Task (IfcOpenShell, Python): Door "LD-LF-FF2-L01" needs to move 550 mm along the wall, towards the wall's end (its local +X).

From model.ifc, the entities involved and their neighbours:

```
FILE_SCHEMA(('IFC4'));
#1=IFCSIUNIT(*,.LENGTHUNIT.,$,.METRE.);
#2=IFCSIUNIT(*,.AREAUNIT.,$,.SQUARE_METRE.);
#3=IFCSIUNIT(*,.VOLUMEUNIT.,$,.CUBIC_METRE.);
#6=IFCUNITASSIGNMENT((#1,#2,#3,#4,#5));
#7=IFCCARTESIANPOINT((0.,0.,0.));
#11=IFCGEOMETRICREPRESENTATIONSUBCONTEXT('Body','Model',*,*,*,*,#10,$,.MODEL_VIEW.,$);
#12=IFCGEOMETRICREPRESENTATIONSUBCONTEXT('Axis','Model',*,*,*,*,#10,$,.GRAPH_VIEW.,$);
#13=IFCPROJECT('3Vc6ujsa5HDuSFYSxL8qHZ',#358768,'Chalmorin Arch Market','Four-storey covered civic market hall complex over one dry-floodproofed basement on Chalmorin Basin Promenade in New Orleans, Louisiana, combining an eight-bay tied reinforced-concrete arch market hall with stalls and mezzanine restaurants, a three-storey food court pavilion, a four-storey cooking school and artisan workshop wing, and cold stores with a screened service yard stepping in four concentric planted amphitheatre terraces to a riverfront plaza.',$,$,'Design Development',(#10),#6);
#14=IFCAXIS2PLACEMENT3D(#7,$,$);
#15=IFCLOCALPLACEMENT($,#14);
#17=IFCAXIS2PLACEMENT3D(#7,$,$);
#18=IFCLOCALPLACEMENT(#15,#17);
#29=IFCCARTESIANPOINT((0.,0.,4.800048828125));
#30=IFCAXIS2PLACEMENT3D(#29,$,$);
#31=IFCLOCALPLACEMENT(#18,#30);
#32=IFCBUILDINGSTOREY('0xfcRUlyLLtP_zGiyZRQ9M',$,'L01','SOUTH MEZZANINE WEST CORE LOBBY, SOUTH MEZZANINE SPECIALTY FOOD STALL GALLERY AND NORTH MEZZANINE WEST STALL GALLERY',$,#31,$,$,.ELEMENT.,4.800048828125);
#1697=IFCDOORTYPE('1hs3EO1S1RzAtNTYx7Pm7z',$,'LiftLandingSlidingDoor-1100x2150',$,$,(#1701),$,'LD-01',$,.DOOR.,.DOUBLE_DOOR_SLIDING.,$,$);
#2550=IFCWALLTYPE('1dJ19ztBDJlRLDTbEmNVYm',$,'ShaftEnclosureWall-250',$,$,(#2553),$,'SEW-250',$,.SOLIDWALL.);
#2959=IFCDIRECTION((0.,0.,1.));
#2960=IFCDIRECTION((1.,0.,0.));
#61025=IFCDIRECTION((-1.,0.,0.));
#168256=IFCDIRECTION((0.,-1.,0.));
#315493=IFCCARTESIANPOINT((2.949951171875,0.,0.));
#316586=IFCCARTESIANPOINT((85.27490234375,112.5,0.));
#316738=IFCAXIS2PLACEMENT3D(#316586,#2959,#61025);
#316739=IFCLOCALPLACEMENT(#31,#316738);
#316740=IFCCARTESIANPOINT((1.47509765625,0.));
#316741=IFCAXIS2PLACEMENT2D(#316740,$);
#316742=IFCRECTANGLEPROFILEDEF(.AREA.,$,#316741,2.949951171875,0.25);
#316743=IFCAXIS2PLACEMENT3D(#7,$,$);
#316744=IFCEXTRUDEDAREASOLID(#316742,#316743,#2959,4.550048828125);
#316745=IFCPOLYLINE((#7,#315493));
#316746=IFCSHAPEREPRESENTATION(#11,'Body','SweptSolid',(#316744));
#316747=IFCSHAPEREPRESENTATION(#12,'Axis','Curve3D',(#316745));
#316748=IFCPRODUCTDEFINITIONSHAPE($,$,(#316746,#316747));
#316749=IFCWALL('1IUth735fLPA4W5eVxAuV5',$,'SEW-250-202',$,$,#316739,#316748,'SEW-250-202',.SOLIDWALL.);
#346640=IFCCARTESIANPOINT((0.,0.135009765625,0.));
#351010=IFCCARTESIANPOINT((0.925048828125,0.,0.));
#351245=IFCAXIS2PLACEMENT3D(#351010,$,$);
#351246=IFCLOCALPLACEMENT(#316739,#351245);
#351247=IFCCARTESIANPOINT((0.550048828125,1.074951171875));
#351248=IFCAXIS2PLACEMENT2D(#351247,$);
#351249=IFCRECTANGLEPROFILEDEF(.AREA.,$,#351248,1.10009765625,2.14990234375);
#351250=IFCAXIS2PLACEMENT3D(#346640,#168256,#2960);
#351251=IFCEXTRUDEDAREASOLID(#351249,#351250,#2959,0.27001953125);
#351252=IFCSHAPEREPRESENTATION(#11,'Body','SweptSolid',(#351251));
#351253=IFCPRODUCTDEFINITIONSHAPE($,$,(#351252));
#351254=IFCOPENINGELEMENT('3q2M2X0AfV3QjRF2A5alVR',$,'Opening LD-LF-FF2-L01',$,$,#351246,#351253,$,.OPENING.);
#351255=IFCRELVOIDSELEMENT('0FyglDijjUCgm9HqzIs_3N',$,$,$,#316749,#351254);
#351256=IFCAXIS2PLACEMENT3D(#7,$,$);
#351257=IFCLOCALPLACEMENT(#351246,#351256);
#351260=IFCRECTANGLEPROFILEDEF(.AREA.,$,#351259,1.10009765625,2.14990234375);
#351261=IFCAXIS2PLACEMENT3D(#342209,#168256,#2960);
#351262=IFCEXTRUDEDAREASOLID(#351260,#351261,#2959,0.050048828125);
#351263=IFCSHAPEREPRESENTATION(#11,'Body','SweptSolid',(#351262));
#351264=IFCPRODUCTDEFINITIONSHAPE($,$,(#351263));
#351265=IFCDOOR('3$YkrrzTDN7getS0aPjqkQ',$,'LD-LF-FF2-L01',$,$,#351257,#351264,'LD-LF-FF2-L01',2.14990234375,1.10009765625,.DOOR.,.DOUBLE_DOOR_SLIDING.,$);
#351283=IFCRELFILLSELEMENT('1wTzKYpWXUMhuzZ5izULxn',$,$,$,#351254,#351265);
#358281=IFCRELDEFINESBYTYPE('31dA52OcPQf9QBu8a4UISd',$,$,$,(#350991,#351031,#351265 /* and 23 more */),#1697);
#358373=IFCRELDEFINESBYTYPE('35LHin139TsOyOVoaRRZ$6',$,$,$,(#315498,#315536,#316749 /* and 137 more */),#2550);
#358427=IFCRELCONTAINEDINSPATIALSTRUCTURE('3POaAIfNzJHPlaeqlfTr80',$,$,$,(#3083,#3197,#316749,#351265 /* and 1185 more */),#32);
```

```python
import ifcopenshell
import ifcopenshell.api.geometry
import ifcopenshell.util.placement
import ifcopenshell.util.unit

model = ifcopenshell.open("model.ifc")
unit_scale = ifcopenshell.util.unit.calculate_unit_scale(model)

door = model.by_guid("3$YkrrzTDN7getS0aPjqkQ")
opening = door.FillsVoids[0].RelatingOpeningElement
wall = opening.VoidsElements[0].RelatingBuildingElement

wall_matrix = ifcopenshell.util.placement.get_local_placement(wall.ObjectPlacement)
shift = wall_matrix[:3, 0] * 0.55 / unit_scale
before = ifcopenshell.util.placement.get_local_placement(door.ObjectPlacement)[:3, 3].copy()

# The door is placed relative to its opening, so it follows when the opening moves.
matrix = ifcopenshell.util.placement.get_local_placement(opening.ObjectPlacement)
matrix[:3, 3] += shift
ifcopenshell.api.geometry.edit_object_placement(
    model, product=opening, matrix=matrix, is_si=False, should_transform_children=True
)

after = ifcopenshell.util.placement.get_local_placement(door.ObjectPlacement)[:3, 3]
print("door moved by", (after - before).round(3) + 0.0)

model.write("model_v2.ifc")
```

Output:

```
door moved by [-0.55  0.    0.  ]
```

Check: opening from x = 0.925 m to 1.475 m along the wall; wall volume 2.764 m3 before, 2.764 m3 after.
